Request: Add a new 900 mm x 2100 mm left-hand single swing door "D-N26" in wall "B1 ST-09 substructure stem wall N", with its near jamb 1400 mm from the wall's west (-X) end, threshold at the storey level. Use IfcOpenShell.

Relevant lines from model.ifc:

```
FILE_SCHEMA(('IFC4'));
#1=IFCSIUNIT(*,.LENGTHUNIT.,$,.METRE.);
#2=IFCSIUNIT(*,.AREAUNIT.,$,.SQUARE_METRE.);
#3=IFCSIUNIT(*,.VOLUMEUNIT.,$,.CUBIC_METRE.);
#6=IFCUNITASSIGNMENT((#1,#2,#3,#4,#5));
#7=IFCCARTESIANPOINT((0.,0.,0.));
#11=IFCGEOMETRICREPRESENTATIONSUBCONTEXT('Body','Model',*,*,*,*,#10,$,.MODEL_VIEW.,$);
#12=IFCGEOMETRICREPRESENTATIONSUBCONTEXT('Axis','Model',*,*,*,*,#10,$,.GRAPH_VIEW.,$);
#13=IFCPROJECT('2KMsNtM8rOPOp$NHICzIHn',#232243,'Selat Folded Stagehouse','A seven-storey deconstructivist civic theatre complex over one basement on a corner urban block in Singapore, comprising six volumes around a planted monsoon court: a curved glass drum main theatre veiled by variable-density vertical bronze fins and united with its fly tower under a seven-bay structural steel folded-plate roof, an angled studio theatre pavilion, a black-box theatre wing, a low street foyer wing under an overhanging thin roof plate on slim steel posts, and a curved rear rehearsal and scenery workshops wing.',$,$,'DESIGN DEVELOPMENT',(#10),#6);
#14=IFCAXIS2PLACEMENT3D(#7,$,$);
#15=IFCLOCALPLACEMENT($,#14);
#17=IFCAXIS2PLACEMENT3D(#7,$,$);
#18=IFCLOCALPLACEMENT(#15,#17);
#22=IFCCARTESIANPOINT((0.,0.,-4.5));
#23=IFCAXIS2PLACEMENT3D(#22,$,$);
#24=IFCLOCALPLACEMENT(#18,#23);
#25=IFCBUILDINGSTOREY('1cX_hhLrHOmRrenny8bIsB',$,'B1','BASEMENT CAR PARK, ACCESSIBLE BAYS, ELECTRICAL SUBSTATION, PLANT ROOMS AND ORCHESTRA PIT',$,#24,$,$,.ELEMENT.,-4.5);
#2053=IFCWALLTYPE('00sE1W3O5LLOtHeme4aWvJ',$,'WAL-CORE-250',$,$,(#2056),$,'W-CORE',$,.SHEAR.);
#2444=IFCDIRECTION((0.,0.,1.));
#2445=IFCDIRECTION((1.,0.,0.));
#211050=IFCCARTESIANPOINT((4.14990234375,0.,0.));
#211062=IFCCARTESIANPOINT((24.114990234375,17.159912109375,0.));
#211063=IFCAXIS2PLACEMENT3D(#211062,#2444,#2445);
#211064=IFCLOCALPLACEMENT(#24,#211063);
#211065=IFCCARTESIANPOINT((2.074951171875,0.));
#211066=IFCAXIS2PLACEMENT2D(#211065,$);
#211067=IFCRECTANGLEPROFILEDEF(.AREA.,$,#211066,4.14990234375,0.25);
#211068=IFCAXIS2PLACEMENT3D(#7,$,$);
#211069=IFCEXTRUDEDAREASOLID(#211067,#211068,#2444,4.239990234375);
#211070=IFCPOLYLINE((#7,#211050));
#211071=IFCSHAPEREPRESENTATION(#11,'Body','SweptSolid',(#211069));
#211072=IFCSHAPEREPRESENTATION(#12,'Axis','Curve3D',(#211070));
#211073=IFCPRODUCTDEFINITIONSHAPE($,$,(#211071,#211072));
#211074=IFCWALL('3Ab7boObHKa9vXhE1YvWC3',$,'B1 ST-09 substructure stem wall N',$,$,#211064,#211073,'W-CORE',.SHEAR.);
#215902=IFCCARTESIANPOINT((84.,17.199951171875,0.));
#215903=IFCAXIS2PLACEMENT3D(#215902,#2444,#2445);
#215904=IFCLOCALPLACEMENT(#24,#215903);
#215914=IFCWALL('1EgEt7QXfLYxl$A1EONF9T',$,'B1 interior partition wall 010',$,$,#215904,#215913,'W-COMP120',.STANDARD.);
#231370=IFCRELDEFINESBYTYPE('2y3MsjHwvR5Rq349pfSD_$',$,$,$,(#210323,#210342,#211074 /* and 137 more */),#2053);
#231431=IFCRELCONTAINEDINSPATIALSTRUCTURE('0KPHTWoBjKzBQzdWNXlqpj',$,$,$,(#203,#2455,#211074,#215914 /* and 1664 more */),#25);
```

```python
import numpy as np
import ifcopenshell
import ifcopenshell.api.feature
import ifcopenshell.api.geometry
import ifcopenshell.api.root
import ifcopenshell.api.spatial
import ifcopenshell.geom
import ifcopenshell.util.element
import ifcopenshell.util.placement
import ifcopenshell.util.representation
import ifcopenshell.util.shape
import ifcopenshell.util.unit

model = ifcopenshell.open("model.ifc")
unit_scale = ifcopenshell.util.unit.calculate_unit_scale(model)
settings = ifcopenshell.geom.settings()


def volume(element):
    """Net volume in cubic metres, openings subtracted."""
    shape = ifcopenshell.geom.create_shape(settings, element)
    return ifcopenshell.util.shape.get_volume(shape.geometry)


wall = model.by_guid("3Ab7boObHKa9vXhE1YvWC3")
storey = ifcopenshell.util.element.get_container(wall, ifc_class="IfcBuildingStorey")
context = ifcopenshell.util.representation.get_context(model, "Model", "Body", "MODEL_VIEW")
before = volume(wall)

width, height, from_end, sill = 0.9, 2.1, 1.4, 0.0  # metres

# The wall runs along its own X axis, and the end named is its -X end.
wall_shape = ifcopenshell.geom.create_shape(settings, wall)
x, y, z = ifcopenshell.util.shape.get_vertices(wall_shape.geometry).T
start = x.min() + from_end
face, thickness = float(y.min()), float(y.max() - y.min())
wall_matrix = ifcopenshell.util.placement.get_local_placement(wall.ObjectPlacement)
level = ifcopenshell.util.placement.get_local_placement(storey.ObjectPlacement)[2, 3]


def in_wall(x, y):
    """Placement at x, y metres in the wall's axes, at sill height."""
    matrix = wall_matrix.copy()
    matrix[:, 3] = wall_matrix @ np.array([x / unit_scale, y / unit_scale, 0.0, 1.0])
    matrix[2, 3] = level + sill / unit_scale
    return matrix


# Opening: a box that overshoots both wall faces by 50 mm.
opening = ifcopenshell.api.root.create_entity(model, ifc_class="IfcOpeningElement", predefined_type="OPENING")
box = ifcopenshell.api.geometry.add_wall_representation(
    model, context=context, length=width, height=height, thickness=thickness + 0.1
)
ifcopenshell.api.geometry.assign_representation(model, product=opening, representation=box)
ifcopenshell.api.geometry.edit_object_placement(model, product=opening, matrix=in_wall(start, face - 0.05), is_si=False)
ifcopenshell.api.feature.add_feature(model, feature=opening, element=wall)

door = ifcopenshell.api.root.create_entity(model, ifc_class="IfcDoor", name="D-N26", predefined_type="DOOR")
door.OverallWidth, door.OverallHeight = width / unit_scale, height / unit_scale
door.OperationType = "SINGLE_SWING_LEFT"
body = ifcopenshell.api.geometry.add_door_representation(
    model,
    context=context,
    overall_width=door.OverallWidth,
    overall_height=door.OverallHeight,
    operation_type="SINGLE_SWING_LEFT",
    lining_properties={"LiningDepth": thickness / unit_scale, "ThresholdDepth": thickness / unit_scale},
)
ifcopenshell.api.geometry.assign_representation(model, product=door, representation=body)
ifcopenshell.api.spatial.assign_container(model, products=[door], relating_structure=storey)
ifcopenshell.api.feature.add_filling(model, opening=opening, element=door)

# The lining spans the wall, so the door starts at the wall face.
ifcopenshell.api.geometry.edit_object_placement(model, product=door, matrix=in_wall(start, face), is_si=False)

after = volume(wall)

print(f"wall volume {before:.3f} -> {after:.3f} m3")

model.write("model_updated.ifc")
```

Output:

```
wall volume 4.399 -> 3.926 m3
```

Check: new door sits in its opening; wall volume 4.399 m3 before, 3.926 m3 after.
